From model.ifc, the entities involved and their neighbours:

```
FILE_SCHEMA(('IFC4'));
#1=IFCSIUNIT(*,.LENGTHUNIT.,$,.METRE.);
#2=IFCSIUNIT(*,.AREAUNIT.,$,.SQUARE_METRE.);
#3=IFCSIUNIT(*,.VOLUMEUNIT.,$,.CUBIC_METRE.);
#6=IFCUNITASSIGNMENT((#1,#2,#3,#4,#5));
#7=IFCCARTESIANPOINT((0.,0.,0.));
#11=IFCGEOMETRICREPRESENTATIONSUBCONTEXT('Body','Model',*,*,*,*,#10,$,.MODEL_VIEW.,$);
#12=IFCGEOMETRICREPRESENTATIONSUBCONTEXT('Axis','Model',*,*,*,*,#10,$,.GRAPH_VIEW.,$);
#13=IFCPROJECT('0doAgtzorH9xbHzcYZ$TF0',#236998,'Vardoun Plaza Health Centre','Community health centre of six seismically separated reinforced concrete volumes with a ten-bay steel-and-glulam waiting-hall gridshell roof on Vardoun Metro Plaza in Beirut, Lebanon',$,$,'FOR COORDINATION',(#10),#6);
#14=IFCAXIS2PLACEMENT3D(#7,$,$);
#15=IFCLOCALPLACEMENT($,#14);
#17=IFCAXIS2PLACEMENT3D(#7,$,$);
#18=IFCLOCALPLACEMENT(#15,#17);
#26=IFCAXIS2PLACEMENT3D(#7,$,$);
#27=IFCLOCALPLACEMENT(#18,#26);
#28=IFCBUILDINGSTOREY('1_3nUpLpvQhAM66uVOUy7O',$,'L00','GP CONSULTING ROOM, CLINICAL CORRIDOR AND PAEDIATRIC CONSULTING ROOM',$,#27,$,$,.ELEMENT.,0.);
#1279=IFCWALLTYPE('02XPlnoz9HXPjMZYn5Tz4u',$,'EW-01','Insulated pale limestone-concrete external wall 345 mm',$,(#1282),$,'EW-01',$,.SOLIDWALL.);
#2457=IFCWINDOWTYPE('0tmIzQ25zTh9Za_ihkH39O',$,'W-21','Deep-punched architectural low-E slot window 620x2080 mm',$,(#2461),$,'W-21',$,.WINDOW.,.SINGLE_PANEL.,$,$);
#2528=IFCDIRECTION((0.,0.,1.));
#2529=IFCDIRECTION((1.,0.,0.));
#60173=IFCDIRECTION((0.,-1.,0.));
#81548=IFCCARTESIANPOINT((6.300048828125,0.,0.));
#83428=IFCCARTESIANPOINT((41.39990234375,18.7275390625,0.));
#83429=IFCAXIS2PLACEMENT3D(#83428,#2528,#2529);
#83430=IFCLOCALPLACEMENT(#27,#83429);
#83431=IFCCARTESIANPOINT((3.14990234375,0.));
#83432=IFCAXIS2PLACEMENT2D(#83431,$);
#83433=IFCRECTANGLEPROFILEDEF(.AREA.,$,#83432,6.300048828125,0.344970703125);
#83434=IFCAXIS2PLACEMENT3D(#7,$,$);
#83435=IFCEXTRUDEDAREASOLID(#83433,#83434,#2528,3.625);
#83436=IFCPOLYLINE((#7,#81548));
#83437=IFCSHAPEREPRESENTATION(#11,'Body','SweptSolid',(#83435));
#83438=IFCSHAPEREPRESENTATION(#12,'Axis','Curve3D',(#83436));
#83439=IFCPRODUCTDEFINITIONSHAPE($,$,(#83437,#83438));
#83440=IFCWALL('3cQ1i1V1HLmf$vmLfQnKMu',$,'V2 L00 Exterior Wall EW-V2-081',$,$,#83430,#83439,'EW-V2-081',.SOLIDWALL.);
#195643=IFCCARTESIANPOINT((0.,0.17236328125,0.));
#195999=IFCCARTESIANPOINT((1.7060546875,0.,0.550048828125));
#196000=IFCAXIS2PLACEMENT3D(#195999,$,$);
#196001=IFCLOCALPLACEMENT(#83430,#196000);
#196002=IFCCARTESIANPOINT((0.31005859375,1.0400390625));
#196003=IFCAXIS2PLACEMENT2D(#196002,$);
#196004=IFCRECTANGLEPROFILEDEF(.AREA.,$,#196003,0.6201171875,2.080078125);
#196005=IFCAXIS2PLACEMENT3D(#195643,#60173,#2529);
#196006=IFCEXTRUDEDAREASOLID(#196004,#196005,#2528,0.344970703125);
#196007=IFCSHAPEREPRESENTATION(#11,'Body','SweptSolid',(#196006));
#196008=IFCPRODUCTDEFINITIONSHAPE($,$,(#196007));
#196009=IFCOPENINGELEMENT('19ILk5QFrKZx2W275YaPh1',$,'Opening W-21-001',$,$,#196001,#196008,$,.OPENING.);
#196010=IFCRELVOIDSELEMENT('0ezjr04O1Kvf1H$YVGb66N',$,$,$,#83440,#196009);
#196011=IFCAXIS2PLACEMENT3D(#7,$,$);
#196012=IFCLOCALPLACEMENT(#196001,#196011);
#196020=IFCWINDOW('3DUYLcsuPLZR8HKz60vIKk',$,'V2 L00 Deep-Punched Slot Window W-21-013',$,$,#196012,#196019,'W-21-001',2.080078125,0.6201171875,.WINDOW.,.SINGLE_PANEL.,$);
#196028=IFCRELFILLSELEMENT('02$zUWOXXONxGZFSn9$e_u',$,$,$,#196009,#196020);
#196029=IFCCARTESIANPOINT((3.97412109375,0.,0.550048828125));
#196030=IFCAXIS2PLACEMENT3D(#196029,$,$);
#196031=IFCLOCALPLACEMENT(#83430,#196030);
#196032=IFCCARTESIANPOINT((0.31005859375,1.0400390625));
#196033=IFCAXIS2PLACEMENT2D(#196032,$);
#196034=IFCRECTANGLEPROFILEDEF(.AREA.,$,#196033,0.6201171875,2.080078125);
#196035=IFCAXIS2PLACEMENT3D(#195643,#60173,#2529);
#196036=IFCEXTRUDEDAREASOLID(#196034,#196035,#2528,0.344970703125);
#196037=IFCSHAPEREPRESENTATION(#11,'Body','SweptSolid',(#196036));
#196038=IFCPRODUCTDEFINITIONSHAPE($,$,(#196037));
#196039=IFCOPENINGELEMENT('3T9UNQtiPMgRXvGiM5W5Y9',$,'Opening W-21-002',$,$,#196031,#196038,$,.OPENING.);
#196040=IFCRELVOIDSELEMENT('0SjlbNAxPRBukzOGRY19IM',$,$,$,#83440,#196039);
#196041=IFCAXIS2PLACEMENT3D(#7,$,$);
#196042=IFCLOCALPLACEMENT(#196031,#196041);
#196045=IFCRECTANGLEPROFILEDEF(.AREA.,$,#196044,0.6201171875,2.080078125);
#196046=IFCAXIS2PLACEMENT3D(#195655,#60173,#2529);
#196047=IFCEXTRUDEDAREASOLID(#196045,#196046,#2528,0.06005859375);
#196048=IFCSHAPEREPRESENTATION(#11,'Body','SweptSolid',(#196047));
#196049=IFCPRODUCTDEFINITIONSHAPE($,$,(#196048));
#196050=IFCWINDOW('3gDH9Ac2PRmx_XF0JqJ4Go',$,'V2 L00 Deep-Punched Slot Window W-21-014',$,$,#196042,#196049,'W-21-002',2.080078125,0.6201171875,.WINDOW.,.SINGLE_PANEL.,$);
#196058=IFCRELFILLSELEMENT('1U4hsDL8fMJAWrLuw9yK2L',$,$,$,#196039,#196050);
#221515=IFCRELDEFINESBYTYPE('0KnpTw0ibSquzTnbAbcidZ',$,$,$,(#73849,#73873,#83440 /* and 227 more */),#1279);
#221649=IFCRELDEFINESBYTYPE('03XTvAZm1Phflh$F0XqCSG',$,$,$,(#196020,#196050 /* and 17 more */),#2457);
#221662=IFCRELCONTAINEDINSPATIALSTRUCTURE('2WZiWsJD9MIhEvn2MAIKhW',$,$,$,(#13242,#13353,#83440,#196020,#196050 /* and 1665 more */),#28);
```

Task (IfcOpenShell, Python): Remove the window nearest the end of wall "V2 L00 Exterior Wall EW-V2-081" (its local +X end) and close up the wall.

```python
import ifcopenshell
import ifcopenshell.api.feature
import ifcopenshell.api.root
import ifcopenshell.geom
import ifcopenshell.util.shape

model = ifcopenshell.open("model.ifc")
settings = ifcopenshell.geom.settings()


def volume(element):
    """Net volume in cubic metres, openings subtracted."""
    shape = ifcopenshell.geom.create_shape(settings, element)
    return ifcopenshell.util.shape.get_volume(shape.geometry)


window = model.by_guid("3gDH9Ac2PRmx_XF0JqJ4Go")
opening = window.FillsVoids[0].RelatingOpeningElement
wall = opening.VoidsElements[0].RelatingBuildingElement
before = volume(wall)

ifcopenshell.api.root.remove_product(model, product=window)
ifcopenshell.api.feature.remove_feature(model, feature=opening)

after = volume(wall)

print(f"wall volume {before:.3f} -> {after:.3f} m3")

model.write("model_v2.ifc")
```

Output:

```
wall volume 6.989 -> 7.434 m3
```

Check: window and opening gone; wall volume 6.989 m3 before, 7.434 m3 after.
